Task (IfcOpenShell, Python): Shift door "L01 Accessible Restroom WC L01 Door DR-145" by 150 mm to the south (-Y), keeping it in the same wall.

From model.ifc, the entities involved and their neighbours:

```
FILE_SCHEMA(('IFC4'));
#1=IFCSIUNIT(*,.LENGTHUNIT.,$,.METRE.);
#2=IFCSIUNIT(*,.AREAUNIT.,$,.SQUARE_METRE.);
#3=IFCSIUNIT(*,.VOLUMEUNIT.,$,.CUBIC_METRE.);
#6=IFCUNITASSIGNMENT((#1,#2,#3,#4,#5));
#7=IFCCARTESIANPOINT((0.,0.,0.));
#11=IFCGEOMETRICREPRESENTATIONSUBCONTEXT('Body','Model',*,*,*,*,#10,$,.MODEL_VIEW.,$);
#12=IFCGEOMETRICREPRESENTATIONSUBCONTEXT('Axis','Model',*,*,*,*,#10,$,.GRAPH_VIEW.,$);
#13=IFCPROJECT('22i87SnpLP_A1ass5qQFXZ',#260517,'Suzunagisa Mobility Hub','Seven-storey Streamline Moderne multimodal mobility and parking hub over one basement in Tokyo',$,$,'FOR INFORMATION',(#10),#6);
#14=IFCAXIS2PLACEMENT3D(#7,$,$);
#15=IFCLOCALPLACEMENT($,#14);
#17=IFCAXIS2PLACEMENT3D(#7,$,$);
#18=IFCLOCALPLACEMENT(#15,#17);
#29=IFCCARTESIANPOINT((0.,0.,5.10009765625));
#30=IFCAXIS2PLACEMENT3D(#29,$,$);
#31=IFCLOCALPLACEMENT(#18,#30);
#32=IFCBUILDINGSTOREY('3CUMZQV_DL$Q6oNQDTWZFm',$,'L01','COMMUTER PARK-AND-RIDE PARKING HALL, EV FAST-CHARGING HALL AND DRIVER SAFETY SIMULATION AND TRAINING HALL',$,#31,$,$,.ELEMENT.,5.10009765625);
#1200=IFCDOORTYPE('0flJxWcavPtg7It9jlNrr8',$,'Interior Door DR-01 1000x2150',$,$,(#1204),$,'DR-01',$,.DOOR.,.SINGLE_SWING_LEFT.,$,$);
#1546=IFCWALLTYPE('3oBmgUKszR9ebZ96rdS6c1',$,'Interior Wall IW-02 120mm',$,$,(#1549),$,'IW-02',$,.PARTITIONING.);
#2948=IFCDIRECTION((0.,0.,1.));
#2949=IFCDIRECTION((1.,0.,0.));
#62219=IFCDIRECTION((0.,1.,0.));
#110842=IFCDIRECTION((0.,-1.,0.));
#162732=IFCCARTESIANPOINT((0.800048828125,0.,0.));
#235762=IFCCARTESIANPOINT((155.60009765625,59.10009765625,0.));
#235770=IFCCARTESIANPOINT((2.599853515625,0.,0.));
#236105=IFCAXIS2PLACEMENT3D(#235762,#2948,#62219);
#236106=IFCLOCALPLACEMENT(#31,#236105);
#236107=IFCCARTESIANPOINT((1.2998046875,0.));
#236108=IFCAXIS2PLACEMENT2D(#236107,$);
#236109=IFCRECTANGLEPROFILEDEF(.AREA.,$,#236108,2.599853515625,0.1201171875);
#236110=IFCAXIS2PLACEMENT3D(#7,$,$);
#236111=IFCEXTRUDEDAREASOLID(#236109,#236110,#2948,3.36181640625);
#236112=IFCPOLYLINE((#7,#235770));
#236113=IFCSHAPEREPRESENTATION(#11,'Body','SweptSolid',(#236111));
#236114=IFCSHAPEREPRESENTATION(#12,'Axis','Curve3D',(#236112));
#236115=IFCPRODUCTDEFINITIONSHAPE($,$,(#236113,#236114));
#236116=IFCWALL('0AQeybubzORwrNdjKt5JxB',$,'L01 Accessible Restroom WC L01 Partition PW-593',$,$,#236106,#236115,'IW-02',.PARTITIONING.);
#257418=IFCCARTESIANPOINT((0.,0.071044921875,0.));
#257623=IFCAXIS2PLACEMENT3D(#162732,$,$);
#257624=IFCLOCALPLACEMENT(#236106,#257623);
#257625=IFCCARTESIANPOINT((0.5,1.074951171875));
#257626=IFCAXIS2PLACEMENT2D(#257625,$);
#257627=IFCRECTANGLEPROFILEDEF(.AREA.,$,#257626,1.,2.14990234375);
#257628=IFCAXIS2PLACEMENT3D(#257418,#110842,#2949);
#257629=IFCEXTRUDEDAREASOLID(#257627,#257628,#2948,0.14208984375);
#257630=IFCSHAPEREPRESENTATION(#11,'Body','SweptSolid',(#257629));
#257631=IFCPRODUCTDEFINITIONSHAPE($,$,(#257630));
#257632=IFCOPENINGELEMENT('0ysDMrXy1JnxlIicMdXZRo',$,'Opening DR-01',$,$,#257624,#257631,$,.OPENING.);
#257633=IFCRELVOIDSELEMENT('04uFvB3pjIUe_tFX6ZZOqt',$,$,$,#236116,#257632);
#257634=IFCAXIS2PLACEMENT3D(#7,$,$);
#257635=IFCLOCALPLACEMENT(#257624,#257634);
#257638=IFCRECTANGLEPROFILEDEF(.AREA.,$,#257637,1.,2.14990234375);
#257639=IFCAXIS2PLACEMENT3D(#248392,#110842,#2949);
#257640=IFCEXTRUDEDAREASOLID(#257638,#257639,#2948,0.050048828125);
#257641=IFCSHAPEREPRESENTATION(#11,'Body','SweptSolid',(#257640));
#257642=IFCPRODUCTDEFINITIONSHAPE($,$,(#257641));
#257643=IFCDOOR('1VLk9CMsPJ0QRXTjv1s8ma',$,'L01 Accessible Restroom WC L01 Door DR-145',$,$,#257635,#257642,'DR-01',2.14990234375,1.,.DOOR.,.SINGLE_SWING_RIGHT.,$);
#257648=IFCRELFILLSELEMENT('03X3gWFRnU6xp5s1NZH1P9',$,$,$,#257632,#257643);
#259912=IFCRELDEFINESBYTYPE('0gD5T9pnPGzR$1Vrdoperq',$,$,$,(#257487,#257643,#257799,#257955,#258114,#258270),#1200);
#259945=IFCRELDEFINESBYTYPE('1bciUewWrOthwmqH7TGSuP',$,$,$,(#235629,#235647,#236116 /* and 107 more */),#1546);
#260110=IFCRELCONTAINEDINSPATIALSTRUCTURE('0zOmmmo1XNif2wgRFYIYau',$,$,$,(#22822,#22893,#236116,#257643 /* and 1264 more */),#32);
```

```python
import ifcopenshell
import ifcopenshell.api.geometry
import ifcopenshell.util.placement
import ifcopenshell.util.unit

model = ifcopenshell.open("model.ifc")
unit_scale = ifcopenshell.util.unit.calculate_unit_scale(model)

door = model.by_guid("1VLk9CMsPJ0QRXTjv1s8ma")
opening = door.FillsVoids[0].RelatingOpeningElement
wall = opening.VoidsElements[0].RelatingBuildingElement

wall_matrix = ifcopenshell.util.placement.get_local_placement(wall.ObjectPlacement)
shift = wall_matrix[:3, 0] * -0.15 / unit_scale
before = ifcopenshell.util.placement.get_local_placement(door.ObjectPlacement)[:3, 3].copy()

# The door is placed relative to its opening, so it follows when the opening moves.
matrix = ifcopenshell.util.placement.get_local_placement(opening.ObjectPlacement)
matrix[:3, 3] += shift
ifcopenshell.api.geometry.edit_object_placement(
    model, product=opening, matrix=matrix, is_si=False, should_transform_children=True
)

after = ifcopenshell.util.placement.get_local_placement(door.ObjectPlacement)[:3, 3]
print("door moved by", (after - before).round(3) + 0.0)

model.write("model_updated.ifc")
```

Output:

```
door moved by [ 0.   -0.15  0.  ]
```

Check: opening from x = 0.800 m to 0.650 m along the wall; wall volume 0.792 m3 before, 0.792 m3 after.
